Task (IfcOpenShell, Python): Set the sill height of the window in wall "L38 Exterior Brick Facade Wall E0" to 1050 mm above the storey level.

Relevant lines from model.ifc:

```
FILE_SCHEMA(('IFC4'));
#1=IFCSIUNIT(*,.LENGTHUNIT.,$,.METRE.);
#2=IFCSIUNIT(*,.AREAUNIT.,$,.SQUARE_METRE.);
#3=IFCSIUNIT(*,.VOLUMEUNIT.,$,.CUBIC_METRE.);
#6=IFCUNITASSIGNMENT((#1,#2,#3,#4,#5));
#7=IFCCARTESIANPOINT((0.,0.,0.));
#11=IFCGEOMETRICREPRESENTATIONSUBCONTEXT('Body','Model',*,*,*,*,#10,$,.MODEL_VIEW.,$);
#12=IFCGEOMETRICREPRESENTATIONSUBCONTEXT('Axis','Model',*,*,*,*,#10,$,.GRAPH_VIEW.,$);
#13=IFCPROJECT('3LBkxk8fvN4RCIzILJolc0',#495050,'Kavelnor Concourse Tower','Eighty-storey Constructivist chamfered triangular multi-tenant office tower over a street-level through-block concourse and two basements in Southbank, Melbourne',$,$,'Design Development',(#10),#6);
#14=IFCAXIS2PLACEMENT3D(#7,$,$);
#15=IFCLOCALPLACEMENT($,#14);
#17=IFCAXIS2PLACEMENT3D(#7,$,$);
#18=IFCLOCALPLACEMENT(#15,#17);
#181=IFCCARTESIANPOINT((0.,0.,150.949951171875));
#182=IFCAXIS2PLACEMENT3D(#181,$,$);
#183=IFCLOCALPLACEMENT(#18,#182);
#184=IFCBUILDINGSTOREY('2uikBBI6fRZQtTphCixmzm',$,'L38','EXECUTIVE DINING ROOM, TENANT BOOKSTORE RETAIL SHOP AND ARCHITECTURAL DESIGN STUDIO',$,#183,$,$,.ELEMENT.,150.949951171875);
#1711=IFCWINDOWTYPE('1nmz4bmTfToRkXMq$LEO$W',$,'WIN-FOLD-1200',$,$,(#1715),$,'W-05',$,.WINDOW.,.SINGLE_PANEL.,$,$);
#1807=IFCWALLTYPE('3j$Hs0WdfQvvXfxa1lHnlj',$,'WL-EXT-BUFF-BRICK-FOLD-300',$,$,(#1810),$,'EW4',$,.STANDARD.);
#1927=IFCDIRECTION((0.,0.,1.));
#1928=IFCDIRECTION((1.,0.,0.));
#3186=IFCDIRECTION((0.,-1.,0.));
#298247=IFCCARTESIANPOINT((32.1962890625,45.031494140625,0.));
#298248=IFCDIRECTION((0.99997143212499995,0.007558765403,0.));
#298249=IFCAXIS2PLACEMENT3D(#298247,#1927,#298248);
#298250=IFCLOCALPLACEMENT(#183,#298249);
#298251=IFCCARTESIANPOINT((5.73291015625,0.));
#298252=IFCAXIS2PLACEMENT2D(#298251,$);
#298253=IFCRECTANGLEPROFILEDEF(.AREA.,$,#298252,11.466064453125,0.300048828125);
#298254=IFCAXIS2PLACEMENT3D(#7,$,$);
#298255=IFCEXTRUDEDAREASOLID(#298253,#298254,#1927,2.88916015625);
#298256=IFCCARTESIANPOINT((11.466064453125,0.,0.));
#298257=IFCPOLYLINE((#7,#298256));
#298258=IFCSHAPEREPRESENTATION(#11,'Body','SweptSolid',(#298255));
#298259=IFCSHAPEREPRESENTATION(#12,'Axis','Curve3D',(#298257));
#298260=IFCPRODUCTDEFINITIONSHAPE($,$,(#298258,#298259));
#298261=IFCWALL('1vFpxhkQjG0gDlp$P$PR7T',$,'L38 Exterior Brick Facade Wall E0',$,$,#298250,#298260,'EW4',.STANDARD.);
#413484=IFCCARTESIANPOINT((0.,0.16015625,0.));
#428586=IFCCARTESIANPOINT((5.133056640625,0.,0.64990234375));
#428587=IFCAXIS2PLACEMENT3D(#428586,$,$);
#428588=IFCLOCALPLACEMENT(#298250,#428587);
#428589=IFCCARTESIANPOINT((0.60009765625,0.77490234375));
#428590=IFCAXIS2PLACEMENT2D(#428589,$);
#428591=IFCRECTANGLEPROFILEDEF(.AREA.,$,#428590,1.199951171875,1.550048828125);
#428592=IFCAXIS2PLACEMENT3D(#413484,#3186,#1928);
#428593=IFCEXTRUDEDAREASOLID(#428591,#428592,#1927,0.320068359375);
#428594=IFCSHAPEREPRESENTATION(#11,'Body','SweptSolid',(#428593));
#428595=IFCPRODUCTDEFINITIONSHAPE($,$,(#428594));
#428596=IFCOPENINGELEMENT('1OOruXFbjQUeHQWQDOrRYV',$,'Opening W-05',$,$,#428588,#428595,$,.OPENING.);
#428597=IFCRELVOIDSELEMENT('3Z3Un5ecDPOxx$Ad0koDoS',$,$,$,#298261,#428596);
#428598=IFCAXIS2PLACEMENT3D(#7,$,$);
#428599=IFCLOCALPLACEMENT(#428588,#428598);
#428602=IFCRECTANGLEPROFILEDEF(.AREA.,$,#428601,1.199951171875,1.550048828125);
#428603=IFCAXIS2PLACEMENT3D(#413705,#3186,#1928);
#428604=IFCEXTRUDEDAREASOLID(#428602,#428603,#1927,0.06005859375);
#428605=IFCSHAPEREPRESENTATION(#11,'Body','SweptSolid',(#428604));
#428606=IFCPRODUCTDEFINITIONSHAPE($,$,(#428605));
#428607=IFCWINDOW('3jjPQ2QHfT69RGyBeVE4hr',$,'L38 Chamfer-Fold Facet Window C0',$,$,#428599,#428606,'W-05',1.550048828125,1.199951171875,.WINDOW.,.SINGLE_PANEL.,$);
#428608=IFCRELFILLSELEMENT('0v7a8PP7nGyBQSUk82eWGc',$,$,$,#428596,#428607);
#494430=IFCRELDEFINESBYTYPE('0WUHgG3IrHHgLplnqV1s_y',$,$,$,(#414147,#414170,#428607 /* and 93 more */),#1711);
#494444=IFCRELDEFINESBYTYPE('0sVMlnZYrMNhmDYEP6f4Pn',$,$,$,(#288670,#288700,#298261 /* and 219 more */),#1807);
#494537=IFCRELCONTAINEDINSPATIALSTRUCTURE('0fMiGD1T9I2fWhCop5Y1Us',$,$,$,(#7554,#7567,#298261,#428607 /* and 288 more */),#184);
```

```python
import numpy as np
import ifcopenshell
import ifcopenshell.api.geometry
import ifcopenshell.geom
import ifcopenshell.util.element
import ifcopenshell.util.placement
import ifcopenshell.util.shape
import ifcopenshell.util.unit

model = ifcopenshell.open("model.ifc")
unit_scale = ifcopenshell.util.unit.calculate_unit_scale(model)

window = model.by_id(428607)
opening = window.FillsVoids[0].RelatingOpeningElement
storey = ifcopenshell.util.element.get_container(window, ifc_class="IfcBuildingStorey")
level = ifcopenshell.util.placement.get_local_placement(storey.ObjectPlacement)[2, 3]

# The opening's origin need not be at the sill, so measure its lowest point.
shape = ifcopenshell.geom.create_shape(ifcopenshell.geom.settings(), opening)
bottom = ifcopenshell.util.shape.get_shape_bottom_elevation(shape, shape.geometry) / unit_scale
dz = level + 1.05 / unit_scale - bottom

shift = np.array([0.0, 0.0, dz])
# The window is placed relative to its opening, so it follows when the opening moves.
matrix = ifcopenshell.util.placement.get_local_placement(opening.ObjectPlacement)
matrix[:3, 3] += shift
ifcopenshell.api.geometry.edit_object_placement(
    model, product=opening, matrix=matrix, is_si=False, should_transform_children=True
)

print(f"moved by {dz * unit_scale:+.3f} m")

model.write("model_v2.ifc")
```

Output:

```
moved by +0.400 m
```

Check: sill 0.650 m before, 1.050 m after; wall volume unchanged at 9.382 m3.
